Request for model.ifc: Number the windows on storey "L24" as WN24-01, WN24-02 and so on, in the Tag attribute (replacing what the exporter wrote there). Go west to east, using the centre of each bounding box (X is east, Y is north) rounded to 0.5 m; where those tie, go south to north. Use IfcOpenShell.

First a look at what the model holds.

```python
import ifcopenshell
import ifcopenshell.util.element
import ifcopenshell.util.placement

model = ifcopenshell.open("model.ifc")
print(model.schema)
storey = next(s for s in model.by_type("IfcBuildingStorey") if s.Name == "L24")
windows = [e for e in ifcopenshell.util.element.get_decomposition(storey) if e.is_a("IfcWindow")]
for e in sorted(windows, key=lambda e: e.id()):
    origin = ifcopenshell.util.placement.get_local_placement(e.ObjectPlacement)[:3, 3]
    print(e.id(), e.Tag, e.Name, origin.round(2) + 0.0, sep=" | ")
```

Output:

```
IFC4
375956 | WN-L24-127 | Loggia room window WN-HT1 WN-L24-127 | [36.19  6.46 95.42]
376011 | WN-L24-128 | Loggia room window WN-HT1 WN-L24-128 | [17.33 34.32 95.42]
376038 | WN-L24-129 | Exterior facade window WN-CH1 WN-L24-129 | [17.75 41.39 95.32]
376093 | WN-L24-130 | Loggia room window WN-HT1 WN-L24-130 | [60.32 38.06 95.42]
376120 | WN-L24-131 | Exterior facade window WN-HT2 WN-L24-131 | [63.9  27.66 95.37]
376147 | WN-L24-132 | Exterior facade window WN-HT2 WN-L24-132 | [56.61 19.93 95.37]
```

```python
import ifcopenshell
import ifcopenshell.geom
import ifcopenshell.util.element
import ifcopenshell.util.shape

model = ifcopenshell.open("model.ifc")
settings = ifcopenshell.geom.settings()
settings.set("use-world-coords", True)


def centre(element):
    shape = ifcopenshell.geom.create_shape(settings, element)
    return ifcopenshell.util.shape.get_bbox_centroid(shape.geometry)


storey = next(s for s in model.by_type("IfcBuildingStorey") if s.Name == "L24")
windows = [e for e in ifcopenshell.util.element.get_decomposition(storey) if e.is_a("IfcWindow")]

# Insertion points can sit at a corner or the storey origin, so sort by the geometry (in metres).
centres = {e: centre(e) for e in windows}
windows.sort(key=lambda e: (round(centres[e][0] / 0.5), centres[e][1]))

for i, e in enumerate(windows, start=1):
    number = f"WN24-{i:02d}"
    e.Tag = number
    print(e.id(), number)

model.write("model_v2.ifc")
```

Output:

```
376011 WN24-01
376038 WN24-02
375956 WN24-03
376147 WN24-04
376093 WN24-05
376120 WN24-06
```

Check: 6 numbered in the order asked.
